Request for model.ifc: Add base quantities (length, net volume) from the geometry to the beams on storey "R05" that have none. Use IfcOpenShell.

First a look at what the model holds.

```python
import ifcopenshell
import ifcopenshell.util.element
import ifcopenshell.util.unit

model = ifcopenshell.open("model.ifc")
print(model.schema)
for unit_type in ("LENGTHUNIT", "AREAUNIT", "VOLUMEUNIT"):
    print(unit_type, ifcopenshell.util.unit.calculate_unit_scale(model, unit_type))
storey = next(s for s in model.by_type("IfcBuildingStorey") if s.Name == "R05")
beams = [e for e in ifcopenshell.util.element.get_decomposition(storey) if e.is_a("IfcBeam")]
for e in sorted(beams, key=lambda e: e.id()):
    print(e.id(), e.is_a(), e.Name, list(ifcopenshell.util.element.get_psets(e, qtos_only=True)), sep=" | ")
```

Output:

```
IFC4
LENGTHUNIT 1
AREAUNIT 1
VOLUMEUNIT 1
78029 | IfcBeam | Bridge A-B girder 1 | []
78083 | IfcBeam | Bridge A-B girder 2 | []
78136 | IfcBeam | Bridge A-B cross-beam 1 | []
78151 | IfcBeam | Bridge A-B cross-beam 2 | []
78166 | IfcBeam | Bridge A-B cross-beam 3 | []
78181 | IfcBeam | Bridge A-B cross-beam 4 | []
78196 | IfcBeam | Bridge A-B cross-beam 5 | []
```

```python
import ifcopenshell
import ifcopenshell.api.pset
import ifcopenshell.geom
import ifcopenshell.util.element
import ifcopenshell.util.shape
import ifcopenshell.util.unit

model = ifcopenshell.open("model.ifc")
unit_scale = ifcopenshell.util.unit.calculate_unit_scale(model)
volume_scale = ifcopenshell.util.unit.calculate_unit_scale(model, "VOLUMEUNIT")
settings = ifcopenshell.geom.settings()

storey = next(s for s in model.by_type("IfcBuildingStorey") if s.Name == "R05")
beams = [e for e in ifcopenshell.util.element.get_decomposition(storey) if e.is_a("IfcBeam")]

for e in sorted(beams, key=lambda e: e.id()):
    if ifcopenshell.util.element.get_psets(e, qtos_only=True, should_inherit=False):
        continue
    # Geometry comes back in metres, in the element's own axes.
    shape = ifcopenshell.geom.create_shape(settings, e)
    values = {
        "Length": ifcopenshell.util.shape.get_max_xyz(shape.geometry) / unit_scale,
        "NetVolume": ifcopenshell.util.shape.get_volume(shape.geometry) / volume_scale,
    }
    qto = ifcopenshell.api.pset.add_qto(model, product=e, name="Qto_BeamBaseQuantities")
    ifcopenshell.api.pset.edit_qto(model, qto=qto, properties=values)
    print(e.id(), {k: round(v, 3) for k, v in values.items()})

model.write("model_rev.ifc")
```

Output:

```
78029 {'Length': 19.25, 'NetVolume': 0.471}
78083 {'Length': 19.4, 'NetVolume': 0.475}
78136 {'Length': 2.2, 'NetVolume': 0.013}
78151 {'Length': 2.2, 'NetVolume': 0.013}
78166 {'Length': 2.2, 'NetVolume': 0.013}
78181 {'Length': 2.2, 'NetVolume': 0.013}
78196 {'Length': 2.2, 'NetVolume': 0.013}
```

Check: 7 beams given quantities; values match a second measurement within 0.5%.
